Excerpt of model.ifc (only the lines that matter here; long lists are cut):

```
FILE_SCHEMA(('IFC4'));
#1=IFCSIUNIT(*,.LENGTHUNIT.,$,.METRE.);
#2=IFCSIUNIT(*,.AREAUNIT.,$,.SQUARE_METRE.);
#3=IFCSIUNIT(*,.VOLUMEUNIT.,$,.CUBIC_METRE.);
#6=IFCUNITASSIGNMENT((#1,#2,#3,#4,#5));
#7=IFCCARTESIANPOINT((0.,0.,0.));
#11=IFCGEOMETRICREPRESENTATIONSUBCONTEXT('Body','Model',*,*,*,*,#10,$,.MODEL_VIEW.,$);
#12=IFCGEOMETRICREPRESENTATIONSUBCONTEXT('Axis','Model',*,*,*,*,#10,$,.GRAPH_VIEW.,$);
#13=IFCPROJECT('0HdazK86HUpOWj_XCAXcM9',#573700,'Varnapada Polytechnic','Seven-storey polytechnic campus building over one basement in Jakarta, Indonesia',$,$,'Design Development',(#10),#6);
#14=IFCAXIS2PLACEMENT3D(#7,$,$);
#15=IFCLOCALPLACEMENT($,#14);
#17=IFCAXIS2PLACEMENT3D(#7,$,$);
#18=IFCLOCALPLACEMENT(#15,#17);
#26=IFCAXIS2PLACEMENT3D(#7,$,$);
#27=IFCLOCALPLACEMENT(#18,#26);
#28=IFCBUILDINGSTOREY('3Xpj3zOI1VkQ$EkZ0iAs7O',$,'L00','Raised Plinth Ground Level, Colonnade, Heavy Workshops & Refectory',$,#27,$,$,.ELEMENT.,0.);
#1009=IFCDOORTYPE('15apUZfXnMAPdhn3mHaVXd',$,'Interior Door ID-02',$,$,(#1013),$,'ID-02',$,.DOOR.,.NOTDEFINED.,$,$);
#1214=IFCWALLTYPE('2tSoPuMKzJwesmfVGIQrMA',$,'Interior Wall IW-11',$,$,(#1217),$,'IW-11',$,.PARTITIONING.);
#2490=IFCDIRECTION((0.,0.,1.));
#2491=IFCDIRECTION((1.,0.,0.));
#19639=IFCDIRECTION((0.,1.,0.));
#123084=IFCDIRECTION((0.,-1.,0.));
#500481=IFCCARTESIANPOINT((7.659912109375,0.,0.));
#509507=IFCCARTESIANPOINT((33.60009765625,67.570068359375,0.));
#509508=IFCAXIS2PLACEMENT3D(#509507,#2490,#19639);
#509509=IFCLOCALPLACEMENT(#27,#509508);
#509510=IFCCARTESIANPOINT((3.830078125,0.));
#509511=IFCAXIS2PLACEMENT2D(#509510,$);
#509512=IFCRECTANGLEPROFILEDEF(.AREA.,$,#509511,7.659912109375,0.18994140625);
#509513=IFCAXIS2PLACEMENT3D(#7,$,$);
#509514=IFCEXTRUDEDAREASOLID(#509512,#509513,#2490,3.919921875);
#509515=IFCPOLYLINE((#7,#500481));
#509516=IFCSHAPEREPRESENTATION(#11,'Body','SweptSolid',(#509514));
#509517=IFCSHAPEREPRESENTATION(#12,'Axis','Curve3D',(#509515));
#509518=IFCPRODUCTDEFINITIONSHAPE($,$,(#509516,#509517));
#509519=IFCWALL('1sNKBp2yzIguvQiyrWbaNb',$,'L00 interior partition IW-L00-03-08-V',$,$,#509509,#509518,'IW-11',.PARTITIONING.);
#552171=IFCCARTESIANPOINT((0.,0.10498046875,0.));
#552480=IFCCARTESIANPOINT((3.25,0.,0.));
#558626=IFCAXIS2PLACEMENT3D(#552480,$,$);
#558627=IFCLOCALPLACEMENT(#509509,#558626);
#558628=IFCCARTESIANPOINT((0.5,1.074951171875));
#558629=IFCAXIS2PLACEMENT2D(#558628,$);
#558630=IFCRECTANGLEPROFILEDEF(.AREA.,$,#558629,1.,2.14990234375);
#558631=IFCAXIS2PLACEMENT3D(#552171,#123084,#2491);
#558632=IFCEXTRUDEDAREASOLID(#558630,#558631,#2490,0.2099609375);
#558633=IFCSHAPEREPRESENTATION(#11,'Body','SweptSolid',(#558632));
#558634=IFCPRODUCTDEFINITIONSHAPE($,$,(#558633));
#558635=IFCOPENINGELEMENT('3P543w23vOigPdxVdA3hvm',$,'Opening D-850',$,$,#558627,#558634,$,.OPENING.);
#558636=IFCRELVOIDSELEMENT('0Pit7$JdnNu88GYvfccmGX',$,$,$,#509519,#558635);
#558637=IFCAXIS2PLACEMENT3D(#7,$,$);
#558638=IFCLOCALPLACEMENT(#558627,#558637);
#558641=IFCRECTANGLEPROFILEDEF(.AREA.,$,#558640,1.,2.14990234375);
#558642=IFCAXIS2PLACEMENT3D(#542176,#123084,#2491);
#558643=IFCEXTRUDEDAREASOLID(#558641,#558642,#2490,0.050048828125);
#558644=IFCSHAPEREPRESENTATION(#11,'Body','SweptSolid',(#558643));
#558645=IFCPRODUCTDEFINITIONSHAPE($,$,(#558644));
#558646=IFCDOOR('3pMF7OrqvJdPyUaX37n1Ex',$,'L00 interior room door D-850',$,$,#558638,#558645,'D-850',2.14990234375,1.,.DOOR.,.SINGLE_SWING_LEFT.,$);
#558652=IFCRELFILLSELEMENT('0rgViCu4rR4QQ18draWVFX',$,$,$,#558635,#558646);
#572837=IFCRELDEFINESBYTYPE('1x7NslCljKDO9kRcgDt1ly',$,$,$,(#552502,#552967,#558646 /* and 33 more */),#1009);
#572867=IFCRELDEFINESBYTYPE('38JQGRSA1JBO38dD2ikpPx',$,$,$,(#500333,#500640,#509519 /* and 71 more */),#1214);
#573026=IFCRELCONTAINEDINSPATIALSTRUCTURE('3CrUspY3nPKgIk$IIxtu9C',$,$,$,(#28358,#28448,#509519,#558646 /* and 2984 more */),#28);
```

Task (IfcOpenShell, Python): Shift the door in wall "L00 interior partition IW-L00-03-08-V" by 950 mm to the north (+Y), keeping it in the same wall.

```python
import ifcopenshell
import ifcopenshell.api.geometry
import ifcopenshell.util.placement

model = ifcopenshell.open("model.ifc")

door = model.by_guid("3pMF7OrqvJdPyUaX37n1Ex")
opening = door.FillsVoids[0].RelatingOpeningElement
wall = opening.VoidsElements[0].RelatingBuildingElement

wall_matrix = ifcopenshell.util.placement.get_local_placement(wall.ObjectPlacement)
shift = wall_matrix[:3, 0] * 0.95
before = ifcopenshell.util.placement.get_local_placement(door.ObjectPlacement)[:3, 3].copy()

# The door is placed relative to its opening, so it follows when the opening moves.
matrix = ifcopenshell.util.placement.get_local_placement(opening.ObjectPlacement)
matrix[:3, 3] += shift
ifcopenshell.api.geometry.edit_object_placement(
    model, product=opening, matrix=matrix, is_si=False, should_transform_children=True
)

after = ifcopenshell.util.placement.get_local_placement(door.ObjectPlacement)[:3, 3]
print("door moved by", (after - before).round(3) + 0.0)

model.write("model_updated.ifc")
```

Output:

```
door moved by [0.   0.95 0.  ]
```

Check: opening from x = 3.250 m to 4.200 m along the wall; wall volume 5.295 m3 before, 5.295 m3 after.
